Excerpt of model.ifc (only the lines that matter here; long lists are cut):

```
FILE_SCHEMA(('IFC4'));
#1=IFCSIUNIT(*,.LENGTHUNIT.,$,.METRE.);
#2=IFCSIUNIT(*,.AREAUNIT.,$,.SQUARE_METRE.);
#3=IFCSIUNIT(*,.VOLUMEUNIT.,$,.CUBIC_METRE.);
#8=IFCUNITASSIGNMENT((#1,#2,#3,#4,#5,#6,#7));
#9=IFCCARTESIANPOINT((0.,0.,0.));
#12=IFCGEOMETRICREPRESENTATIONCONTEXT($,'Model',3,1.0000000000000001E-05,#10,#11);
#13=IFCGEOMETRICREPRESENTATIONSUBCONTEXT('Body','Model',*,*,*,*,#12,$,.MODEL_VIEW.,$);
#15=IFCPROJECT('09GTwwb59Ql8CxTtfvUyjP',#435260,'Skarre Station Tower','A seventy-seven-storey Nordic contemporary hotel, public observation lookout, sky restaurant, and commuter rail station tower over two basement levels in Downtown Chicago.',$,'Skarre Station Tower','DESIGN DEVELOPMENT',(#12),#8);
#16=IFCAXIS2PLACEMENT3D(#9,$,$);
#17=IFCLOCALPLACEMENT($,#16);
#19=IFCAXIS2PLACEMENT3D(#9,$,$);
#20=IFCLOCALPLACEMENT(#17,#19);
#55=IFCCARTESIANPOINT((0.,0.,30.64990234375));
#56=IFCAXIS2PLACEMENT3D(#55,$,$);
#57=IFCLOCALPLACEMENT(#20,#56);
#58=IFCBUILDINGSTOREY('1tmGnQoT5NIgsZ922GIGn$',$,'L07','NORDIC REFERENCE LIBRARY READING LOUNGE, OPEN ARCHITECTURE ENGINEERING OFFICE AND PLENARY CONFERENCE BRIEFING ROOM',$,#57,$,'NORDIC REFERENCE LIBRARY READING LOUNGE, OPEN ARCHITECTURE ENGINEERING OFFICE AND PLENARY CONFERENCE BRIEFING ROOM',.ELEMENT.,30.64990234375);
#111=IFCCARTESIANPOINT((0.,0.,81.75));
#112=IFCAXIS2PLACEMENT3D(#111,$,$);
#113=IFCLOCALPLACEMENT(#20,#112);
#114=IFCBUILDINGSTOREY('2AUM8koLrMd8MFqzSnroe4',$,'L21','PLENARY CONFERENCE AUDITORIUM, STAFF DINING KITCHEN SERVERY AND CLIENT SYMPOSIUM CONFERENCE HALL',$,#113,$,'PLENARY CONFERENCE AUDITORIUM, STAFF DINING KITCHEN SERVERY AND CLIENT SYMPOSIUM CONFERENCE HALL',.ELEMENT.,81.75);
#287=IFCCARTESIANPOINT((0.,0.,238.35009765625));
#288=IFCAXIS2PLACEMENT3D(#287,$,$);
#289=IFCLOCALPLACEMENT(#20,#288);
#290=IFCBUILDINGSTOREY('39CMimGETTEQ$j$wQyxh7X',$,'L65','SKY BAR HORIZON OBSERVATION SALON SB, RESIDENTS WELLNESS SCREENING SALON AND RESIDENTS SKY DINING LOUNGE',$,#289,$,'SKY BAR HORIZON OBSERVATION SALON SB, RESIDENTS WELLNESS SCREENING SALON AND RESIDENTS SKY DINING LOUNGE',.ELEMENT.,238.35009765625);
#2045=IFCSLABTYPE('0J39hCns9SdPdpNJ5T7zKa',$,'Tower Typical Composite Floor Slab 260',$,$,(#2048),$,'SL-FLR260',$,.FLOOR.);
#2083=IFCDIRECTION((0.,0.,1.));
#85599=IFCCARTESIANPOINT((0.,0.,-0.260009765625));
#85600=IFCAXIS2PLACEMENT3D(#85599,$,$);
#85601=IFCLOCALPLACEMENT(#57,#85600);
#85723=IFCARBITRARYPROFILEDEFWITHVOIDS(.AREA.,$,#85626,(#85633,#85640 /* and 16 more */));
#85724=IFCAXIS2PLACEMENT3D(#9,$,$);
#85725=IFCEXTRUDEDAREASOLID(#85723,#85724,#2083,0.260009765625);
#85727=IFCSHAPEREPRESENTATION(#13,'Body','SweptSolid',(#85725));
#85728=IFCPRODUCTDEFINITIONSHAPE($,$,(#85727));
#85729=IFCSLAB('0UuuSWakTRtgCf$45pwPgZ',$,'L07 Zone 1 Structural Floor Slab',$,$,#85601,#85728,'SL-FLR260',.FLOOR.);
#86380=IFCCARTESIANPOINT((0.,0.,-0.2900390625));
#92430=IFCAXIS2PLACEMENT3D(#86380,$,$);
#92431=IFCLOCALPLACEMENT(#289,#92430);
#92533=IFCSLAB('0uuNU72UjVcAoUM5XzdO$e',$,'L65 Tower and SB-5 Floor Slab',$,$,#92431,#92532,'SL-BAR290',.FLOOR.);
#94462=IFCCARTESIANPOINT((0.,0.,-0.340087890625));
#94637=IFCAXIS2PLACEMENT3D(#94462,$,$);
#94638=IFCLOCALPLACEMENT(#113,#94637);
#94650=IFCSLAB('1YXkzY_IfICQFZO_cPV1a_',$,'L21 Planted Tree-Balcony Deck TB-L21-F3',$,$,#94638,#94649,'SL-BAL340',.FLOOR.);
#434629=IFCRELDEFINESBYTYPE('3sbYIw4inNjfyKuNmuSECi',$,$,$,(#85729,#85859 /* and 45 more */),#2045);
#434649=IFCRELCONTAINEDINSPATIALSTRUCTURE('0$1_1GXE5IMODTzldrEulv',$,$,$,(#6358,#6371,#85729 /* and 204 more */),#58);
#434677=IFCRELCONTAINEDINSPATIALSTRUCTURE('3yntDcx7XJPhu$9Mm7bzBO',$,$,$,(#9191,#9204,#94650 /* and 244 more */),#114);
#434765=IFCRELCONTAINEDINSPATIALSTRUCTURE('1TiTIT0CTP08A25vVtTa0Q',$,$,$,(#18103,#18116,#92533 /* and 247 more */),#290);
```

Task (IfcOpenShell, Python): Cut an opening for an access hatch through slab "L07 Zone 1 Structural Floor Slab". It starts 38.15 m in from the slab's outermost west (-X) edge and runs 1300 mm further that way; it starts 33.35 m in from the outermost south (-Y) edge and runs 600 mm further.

```python
import numpy as np
import ifcopenshell
import ifcopenshell.api.feature
import ifcopenshell.api.geometry
import ifcopenshell.api.root
import ifcopenshell.geom
import ifcopenshell.util.placement
import ifcopenshell.util.representation
import ifcopenshell.util.shape
import ifcopenshell.util.unit

model = ifcopenshell.open("model.ifc")
unit_scale = ifcopenshell.util.unit.calculate_unit_scale(model)
settings = ifcopenshell.geom.settings()


def volume(element):
    """Net volume in cubic metres, openings subtracted."""
    shape = ifcopenshell.geom.create_shape(settings, element)
    return ifcopenshell.util.shape.get_volume(shape.geometry)


slab = model.by_guid("0UuuSWakTRtgCf$45pwPgZ")
before = volume(slab)

# Extent in the slab's own axes, in metres. The edges named are its -X and -Y sides.
slab_shape = ifcopenshell.geom.create_shape(settings, slab)
vertices = ifcopenshell.util.shape.get_vertices(slab_shape.geometry)
x_min, y_min, bottom = vertices.min(axis=0)
top = vertices[:, 2].max()

opening = ifcopenshell.api.root.create_entity(model, ifc_class="IfcOpeningElement", name="Access hatch opening", predefined_type="OPENING")
context = ifcopenshell.util.representation.get_context(model, "Model", "Body", "MODEL_VIEW")
width, depth = 1.3, 0.6
outline = [(0.0, 0.0), (width, 0.0), (width, depth), (0.0, depth), (0.0, 0.0)]
# Overshoot both faces by 50 mm so the cut is clean.
shape = ifcopenshell.api.geometry.add_slab_representation(
    model, context=context, depth=top - bottom + 0.1, polyline=outline
)
ifcopenshell.api.geometry.assign_representation(model, product=opening, representation=shape)

matrix = ifcopenshell.util.placement.get_local_placement(slab.ObjectPlacement)
matrix[:, 3] = matrix @ np.append(np.array([x_min + 38.15, y_min + 33.35, bottom - 0.05]) / unit_scale, 1.0)
ifcopenshell.api.geometry.edit_object_placement(model, product=opening, matrix=matrix, is_si=False)
ifcopenshell.api.feature.add_feature(model, feature=opening, element=slab)

after = volume(slab)

print(f"slab volume {before:.3f} -> {after:.3f} m3")

model.write("model_updated.ifc")
```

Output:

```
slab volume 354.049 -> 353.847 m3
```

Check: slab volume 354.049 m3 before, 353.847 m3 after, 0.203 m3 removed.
